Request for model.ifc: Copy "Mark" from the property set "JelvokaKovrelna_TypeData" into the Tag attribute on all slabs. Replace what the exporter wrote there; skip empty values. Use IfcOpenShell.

First a look at what the model holds.

```python
import ifcopenshell
import ifcopenshell.util.element

model = ifcopenshell.open("model.ifc")
print(model.schema)
slabs = model.by_type("IfcSlab")
print(len(slabs), "slabs")
for e in slabs[:8]:
    source = ifcopenshell.util.element.get_pset(e, "JelvokaKovrelna_TypeData", "Mark")
    target = e.Tag
    print(e.id(), repr(source), repr(target), sep=" | ")
```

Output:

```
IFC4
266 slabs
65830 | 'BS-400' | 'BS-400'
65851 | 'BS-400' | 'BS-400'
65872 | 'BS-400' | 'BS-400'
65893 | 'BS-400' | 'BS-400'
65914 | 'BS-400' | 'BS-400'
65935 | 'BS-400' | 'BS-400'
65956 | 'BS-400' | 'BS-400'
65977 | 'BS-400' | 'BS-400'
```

```python
import ifcopenshell
import ifcopenshell.util.element

model = ifcopenshell.open("model.ifc")

count = 0
for e in model.by_type("IfcSlab"):
    value = ifcopenshell.util.element.get_pset(e, "JelvokaKovrelna_TypeData", "Mark")
    current = e.Tag
    if not value or not value.strip() or current == value:
        continue
    e.Tag = value
    count += 1

print(count, "slabs updated")

model.write("model-out.ifc")
```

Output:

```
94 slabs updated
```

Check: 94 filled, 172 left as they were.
